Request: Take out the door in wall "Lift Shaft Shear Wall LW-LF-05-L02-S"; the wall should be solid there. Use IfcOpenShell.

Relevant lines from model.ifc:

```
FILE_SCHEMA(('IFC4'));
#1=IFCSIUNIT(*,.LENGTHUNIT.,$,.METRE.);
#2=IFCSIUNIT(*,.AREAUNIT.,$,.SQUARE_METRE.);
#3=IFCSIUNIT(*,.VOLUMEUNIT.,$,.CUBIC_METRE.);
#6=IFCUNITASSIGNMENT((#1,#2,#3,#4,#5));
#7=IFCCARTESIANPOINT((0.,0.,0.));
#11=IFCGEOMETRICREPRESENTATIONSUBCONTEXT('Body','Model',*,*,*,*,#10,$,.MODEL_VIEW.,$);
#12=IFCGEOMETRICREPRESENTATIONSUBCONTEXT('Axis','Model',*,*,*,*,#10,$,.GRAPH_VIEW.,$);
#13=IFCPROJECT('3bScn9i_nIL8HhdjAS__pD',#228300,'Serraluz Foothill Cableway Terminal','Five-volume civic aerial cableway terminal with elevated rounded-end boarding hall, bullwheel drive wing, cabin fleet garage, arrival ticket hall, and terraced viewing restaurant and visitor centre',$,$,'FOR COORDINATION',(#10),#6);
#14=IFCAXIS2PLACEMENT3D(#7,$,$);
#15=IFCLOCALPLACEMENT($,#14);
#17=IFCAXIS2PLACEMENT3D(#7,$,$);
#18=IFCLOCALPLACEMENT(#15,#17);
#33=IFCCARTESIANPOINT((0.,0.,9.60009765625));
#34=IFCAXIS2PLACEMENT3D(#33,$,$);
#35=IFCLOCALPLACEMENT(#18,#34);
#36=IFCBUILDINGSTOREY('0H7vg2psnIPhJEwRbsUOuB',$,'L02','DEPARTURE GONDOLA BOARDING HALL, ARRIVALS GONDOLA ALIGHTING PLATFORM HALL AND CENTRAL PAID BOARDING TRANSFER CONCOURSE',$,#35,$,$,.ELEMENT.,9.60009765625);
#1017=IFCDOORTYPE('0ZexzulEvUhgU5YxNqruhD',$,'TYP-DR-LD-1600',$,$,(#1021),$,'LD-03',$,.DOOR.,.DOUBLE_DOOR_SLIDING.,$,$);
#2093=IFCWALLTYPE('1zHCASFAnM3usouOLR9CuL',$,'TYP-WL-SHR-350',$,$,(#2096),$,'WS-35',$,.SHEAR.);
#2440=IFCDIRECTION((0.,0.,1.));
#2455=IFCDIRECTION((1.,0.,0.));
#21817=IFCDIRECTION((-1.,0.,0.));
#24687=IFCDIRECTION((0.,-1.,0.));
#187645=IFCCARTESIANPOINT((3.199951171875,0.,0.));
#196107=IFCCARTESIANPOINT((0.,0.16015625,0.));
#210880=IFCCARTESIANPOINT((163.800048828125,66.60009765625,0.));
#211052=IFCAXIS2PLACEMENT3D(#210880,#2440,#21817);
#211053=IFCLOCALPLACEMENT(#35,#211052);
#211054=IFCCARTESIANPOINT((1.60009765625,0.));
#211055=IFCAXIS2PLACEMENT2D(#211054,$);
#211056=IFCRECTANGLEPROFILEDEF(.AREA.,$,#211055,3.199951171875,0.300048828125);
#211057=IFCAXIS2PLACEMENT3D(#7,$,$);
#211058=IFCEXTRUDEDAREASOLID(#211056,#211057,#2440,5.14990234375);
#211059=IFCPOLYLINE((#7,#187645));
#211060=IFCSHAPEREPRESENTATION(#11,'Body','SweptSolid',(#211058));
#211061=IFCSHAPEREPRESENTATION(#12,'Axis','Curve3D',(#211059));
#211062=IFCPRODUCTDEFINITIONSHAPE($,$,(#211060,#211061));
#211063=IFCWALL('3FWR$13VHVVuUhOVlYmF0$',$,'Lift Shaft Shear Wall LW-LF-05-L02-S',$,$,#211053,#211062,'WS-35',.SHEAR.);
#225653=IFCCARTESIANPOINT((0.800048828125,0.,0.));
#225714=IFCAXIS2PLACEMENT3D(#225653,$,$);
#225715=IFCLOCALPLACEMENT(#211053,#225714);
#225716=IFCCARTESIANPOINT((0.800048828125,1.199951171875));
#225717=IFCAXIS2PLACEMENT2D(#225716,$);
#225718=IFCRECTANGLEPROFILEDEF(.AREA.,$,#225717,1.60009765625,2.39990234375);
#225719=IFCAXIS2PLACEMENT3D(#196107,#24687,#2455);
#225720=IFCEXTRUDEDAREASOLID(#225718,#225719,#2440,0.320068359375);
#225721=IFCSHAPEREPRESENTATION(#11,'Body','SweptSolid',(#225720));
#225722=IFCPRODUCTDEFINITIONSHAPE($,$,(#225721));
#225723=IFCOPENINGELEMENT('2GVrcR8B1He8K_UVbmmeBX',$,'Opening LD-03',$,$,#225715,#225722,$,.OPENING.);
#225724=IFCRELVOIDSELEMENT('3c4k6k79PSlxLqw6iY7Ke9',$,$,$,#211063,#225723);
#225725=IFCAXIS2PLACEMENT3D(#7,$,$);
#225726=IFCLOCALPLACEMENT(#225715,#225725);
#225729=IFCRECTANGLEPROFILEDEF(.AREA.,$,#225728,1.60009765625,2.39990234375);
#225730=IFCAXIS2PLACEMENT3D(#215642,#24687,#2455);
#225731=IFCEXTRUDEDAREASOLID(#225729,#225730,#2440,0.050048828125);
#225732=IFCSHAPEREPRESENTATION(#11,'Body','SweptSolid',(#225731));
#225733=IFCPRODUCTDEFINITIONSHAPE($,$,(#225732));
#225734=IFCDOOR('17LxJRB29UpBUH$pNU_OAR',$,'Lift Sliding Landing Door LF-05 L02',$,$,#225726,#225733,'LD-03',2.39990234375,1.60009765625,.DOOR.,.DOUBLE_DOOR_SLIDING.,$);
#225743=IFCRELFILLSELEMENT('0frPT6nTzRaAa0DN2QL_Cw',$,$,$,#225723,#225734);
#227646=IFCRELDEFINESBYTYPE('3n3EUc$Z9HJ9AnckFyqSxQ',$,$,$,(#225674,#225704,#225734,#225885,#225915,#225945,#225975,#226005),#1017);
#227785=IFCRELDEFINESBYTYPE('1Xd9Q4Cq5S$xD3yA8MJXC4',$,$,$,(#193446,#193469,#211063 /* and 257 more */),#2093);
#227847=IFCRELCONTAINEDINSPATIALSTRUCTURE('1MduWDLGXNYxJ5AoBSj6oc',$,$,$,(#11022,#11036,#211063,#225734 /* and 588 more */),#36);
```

```python
import ifcopenshell
import ifcopenshell.api.feature
import ifcopenshell.api.root
import ifcopenshell.geom
import ifcopenshell.util.shape

model = ifcopenshell.open("model.ifc")
settings = ifcopenshell.geom.settings()


def volume(element):
    """Net volume in cubic metres, openings subtracted."""
    shape = ifcopenshell.geom.create_shape(settings, element)
    return ifcopenshell.util.shape.get_volume(shape.geometry)


door = model.by_id(225734)
opening = door.FillsVoids[0].RelatingOpeningElement
wall = opening.VoidsElements[0].RelatingBuildingElement
before = volume(wall)

ifcopenshell.api.root.remove_product(model, product=door)
ifcopenshell.api.feature.remove_feature(model, feature=opening)

after = volume(wall)

print(f"wall volume {before:.3f} -> {after:.3f} m3")

model.write("model_v2.ifc")
```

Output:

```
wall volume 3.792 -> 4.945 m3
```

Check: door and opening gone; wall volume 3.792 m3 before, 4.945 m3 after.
